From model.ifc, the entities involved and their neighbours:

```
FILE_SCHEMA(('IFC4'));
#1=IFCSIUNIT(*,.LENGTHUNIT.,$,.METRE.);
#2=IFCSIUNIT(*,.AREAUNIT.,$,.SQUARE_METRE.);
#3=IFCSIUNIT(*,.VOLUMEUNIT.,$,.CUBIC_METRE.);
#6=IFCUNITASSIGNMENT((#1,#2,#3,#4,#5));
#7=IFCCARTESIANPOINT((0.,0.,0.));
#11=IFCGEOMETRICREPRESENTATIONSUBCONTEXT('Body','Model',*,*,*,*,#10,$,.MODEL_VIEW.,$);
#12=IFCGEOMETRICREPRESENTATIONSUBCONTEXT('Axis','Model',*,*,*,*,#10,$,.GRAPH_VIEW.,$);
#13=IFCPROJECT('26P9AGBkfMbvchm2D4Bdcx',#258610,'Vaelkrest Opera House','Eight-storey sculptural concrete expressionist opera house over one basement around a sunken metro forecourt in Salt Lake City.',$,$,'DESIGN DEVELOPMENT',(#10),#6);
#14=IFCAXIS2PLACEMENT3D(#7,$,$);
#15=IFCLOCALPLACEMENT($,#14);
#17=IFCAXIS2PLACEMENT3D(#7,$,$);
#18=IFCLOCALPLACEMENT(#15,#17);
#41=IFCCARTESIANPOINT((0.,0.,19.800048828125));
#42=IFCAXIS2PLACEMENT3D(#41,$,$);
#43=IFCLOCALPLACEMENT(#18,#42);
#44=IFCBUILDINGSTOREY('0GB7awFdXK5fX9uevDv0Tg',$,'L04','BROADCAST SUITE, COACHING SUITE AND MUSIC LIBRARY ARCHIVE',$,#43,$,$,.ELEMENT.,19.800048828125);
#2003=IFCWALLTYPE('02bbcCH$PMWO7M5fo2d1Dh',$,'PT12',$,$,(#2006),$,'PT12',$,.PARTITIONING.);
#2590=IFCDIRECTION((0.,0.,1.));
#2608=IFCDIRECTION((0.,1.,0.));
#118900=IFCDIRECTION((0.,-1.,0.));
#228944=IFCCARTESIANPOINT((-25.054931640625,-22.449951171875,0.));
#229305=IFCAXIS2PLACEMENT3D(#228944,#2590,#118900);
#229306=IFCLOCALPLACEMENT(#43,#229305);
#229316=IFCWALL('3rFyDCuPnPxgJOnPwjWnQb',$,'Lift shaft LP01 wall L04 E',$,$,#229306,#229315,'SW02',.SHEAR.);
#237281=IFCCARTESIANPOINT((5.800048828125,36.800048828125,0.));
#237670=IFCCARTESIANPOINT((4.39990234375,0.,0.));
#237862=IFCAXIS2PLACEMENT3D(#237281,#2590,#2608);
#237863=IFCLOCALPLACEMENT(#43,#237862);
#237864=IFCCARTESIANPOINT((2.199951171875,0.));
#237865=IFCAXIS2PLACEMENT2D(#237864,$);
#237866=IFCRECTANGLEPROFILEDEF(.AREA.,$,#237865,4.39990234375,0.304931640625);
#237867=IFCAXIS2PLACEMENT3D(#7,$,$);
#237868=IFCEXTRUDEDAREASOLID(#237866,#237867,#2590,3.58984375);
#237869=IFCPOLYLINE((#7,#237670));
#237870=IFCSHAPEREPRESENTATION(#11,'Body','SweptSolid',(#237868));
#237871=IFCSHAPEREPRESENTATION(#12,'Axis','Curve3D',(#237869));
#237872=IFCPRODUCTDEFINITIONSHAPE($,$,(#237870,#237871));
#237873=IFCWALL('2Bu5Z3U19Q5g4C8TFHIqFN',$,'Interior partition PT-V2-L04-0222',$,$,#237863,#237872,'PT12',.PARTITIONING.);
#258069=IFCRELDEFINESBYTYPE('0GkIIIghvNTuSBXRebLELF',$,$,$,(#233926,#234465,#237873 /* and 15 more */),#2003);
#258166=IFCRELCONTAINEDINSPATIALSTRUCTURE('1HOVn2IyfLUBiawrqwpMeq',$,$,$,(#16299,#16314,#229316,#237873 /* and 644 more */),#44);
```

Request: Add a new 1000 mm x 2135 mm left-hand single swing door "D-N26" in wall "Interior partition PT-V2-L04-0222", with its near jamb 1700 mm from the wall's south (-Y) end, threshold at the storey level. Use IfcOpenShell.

```python
import numpy as np
import ifcopenshell
import ifcopenshell.api.feature
import ifcopenshell.api.geometry
import ifcopenshell.api.root
import ifcopenshell.api.spatial
import ifcopenshell.geom
import ifcopenshell.util.element
import ifcopenshell.util.placement
import ifcopenshell.util.representation
import ifcopenshell.util.shape
import ifcopenshell.util.unit

model = ifcopenshell.open("model.ifc")
unit_scale = ifcopenshell.util.unit.calculate_unit_scale(model)
settings = ifcopenshell.geom.settings()


def volume(element):
    """Net volume in cubic metres, openings subtracted."""
    shape = ifcopenshell.geom.create_shape(settings, element)
    return ifcopenshell.util.shape.get_volume(shape.geometry)


wall = model.by_id(237873)
storey = ifcopenshell.util.element.get_container(wall, ifc_class="IfcBuildingStorey")
context = ifcopenshell.util.representation.get_context(model, "Model", "Body", "MODEL_VIEW")
before = volume(wall)

width, height, from_end, sill = 1, 2.135, 1.7, 0.0  # metres

# The wall runs along its own X axis, and the end named is its -X end.
wall_shape = ifcopenshell.geom.create_shape(settings, wall)
x, y, z = ifcopenshell.util.shape.get_vertices(wall_shape.geometry).T
start = x.min() + from_end
face, thickness = float(y.min()), float(y.max() - y.min())
wall_matrix = ifcopenshell.util.placement.get_local_placement(wall.ObjectPlacement)
level = ifcopenshell.util.placement.get_local_placement(storey.ObjectPlacement)[2, 3]


def in_wall(x, y):
    """Placement at x, y metres in the wall's axes, at sill height."""
    matrix = wall_matrix.copy()
    matrix[:, 3] = wall_matrix @ np.array([x / unit_scale, y / unit_scale, 0.0, 1.0])
    matrix[2, 3] = level + sill / unit_scale
    return matrix


# Opening: a box that overshoots both wall faces by 50 mm.
opening = ifcopenshell.api.root.create_entity(model, ifc_class="IfcOpeningElement", predefined_type="OPENING")
box = ifcopenshell.api.geometry.add_wall_representation(
    model, context=context, length=width, height=height, thickness=thickness + 0.1
)
ifcopenshell.api.geometry.assign_representation(model, product=opening, representation=box)
ifcopenshell.api.geometry.edit_object_placement(model, product=opening, matrix=in_wall(start, face - 0.05), is_si=False)
ifcopenshell.api.feature.add_feature(model, feature=opening, element=wall)

door = ifcopenshell.api.root.create_entity(model, ifc_class="IfcDoor", name="D-N26", predefined_type="DOOR")
door.OverallWidth, door.OverallHeight = width / unit_scale, height / unit_scale
door.OperationType = "SINGLE_SWING_LEFT"
body = ifcopenshell.api.geometry.add_door_representation(
    model,
    context=context,
    overall_width=door.OverallWidth,
    overall_height=door.OverallHeight,
    operation_type="SINGLE_SWING_LEFT",
    lining_properties={"LiningDepth": thickness / unit_scale, "ThresholdDepth": thickness / unit_scale},
)
ifcopenshell.api.geometry.assign_representation(model, product=door, representation=body)
ifcopenshell.api.spatial.assign_container(model, products=[door], relating_structure=storey)
ifcopenshell.api.feature.add_filling(model, opening=opening, element=door)

# The lining spans the wall, so the door starts at the wall face.
ifcopenshell.api.geometry.edit_object_placement(model, product=door, matrix=in_wall(start, face), is_si=False)

after = volume(wall)

print(f"wall volume {before:.3f} -> {after:.3f} m3")

model.write("model_edited.ifc")
```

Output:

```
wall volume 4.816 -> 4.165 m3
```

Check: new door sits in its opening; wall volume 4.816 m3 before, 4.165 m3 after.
